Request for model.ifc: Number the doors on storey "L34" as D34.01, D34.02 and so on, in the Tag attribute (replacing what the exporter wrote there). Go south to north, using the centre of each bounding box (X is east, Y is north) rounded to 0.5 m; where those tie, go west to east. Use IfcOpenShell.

First a look at what the model holds.

```python
import ifcopenshell
import ifcopenshell.util.element
import ifcopenshell.util.placement

model = ifcopenshell.open("model.ifc")
print(model.schema)
storey = next(s for s in model.by_type("IfcBuildingStorey") if s.Name == "L34")
doors = [e for e in ifcopenshell.util.element.get_decomposition(storey) if e.is_a("IfcDoor")]
for e in sorted(doors, key=lambda e: e.id()):
    origin = ifcopenshell.util.placement.get_local_placement(e.ObjectPlacement)[:3, 3]
    print(e.id(), e.Tag, e.Name, origin.round(2) + 0.0, sep=" | ")
```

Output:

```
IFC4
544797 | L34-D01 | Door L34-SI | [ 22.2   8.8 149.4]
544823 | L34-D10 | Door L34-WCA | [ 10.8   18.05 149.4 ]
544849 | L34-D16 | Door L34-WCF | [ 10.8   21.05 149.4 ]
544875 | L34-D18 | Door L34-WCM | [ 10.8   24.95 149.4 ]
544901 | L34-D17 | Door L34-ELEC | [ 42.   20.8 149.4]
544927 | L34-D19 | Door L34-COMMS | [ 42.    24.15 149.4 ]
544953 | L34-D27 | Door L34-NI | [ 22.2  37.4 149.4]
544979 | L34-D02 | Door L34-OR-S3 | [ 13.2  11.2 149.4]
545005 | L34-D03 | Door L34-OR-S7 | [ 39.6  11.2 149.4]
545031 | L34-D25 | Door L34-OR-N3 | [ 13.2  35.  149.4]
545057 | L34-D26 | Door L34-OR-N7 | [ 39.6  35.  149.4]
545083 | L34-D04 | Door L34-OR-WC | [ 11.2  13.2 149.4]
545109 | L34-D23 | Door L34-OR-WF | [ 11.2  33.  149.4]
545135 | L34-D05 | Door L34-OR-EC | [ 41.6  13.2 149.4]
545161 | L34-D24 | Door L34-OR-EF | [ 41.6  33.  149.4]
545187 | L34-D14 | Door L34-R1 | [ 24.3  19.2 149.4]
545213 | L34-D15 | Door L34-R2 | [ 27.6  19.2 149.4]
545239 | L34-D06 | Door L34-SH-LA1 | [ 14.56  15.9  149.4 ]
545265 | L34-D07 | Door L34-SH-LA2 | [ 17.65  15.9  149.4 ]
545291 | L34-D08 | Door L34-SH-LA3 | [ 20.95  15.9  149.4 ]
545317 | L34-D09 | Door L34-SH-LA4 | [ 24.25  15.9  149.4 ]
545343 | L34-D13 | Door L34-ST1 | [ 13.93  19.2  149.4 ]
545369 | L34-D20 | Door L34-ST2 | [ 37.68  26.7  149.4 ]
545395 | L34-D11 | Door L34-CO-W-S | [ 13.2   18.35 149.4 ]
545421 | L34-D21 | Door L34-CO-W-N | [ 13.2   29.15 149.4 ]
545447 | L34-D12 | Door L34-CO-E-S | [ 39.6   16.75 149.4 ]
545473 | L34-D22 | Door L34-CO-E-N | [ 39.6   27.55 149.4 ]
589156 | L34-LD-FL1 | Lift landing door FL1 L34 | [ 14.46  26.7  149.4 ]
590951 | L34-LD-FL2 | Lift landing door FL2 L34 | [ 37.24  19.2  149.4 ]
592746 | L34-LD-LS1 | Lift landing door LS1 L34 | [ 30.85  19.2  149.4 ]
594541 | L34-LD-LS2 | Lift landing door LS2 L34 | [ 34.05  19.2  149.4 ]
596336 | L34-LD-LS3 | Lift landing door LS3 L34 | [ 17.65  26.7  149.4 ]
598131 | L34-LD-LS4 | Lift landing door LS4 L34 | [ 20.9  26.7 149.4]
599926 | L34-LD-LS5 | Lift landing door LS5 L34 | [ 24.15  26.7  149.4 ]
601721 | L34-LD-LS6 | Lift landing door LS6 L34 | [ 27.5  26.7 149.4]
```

```python
import ifcopenshell
import ifcopenshell.geom
import ifcopenshell.util.element
import ifcopenshell.util.shape

model = ifcopenshell.open("model.ifc")
settings = ifcopenshell.geom.settings()
settings.set("use-world-coords", True)


def centre(element):
    shape = ifcopenshell.geom.create_shape(settings, element)
    return ifcopenshell.util.shape.get_bbox_centroid(shape.geometry)


storey = next(s for s in model.by_type("IfcBuildingStorey") if s.Name == "L34")
doors = [e for e in ifcopenshell.util.element.get_decomposition(storey) if e.is_a("IfcDoor")]

# Insertion points can sit at a corner or the storey origin, so sort by the geometry (in metres).
centres = {e: centre(e) for e in doors}
doors.sort(key=lambda e: (round(centres[e][1] / 0.5), centres[e][0]))

for i, e in enumerate(doors, start=1):
    number = f"D34.{i:02d}"
    e.Tag = number
    print(e.id(), number)

model.write("model_edited.ifc")
```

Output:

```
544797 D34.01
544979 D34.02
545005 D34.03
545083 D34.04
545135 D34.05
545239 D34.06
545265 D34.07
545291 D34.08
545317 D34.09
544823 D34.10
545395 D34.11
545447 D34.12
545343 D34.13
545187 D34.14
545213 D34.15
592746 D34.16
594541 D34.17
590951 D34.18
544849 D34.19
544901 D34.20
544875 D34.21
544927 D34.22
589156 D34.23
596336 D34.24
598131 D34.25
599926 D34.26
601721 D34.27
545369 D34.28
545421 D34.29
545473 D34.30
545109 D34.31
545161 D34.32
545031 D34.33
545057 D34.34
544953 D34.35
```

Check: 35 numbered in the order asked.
